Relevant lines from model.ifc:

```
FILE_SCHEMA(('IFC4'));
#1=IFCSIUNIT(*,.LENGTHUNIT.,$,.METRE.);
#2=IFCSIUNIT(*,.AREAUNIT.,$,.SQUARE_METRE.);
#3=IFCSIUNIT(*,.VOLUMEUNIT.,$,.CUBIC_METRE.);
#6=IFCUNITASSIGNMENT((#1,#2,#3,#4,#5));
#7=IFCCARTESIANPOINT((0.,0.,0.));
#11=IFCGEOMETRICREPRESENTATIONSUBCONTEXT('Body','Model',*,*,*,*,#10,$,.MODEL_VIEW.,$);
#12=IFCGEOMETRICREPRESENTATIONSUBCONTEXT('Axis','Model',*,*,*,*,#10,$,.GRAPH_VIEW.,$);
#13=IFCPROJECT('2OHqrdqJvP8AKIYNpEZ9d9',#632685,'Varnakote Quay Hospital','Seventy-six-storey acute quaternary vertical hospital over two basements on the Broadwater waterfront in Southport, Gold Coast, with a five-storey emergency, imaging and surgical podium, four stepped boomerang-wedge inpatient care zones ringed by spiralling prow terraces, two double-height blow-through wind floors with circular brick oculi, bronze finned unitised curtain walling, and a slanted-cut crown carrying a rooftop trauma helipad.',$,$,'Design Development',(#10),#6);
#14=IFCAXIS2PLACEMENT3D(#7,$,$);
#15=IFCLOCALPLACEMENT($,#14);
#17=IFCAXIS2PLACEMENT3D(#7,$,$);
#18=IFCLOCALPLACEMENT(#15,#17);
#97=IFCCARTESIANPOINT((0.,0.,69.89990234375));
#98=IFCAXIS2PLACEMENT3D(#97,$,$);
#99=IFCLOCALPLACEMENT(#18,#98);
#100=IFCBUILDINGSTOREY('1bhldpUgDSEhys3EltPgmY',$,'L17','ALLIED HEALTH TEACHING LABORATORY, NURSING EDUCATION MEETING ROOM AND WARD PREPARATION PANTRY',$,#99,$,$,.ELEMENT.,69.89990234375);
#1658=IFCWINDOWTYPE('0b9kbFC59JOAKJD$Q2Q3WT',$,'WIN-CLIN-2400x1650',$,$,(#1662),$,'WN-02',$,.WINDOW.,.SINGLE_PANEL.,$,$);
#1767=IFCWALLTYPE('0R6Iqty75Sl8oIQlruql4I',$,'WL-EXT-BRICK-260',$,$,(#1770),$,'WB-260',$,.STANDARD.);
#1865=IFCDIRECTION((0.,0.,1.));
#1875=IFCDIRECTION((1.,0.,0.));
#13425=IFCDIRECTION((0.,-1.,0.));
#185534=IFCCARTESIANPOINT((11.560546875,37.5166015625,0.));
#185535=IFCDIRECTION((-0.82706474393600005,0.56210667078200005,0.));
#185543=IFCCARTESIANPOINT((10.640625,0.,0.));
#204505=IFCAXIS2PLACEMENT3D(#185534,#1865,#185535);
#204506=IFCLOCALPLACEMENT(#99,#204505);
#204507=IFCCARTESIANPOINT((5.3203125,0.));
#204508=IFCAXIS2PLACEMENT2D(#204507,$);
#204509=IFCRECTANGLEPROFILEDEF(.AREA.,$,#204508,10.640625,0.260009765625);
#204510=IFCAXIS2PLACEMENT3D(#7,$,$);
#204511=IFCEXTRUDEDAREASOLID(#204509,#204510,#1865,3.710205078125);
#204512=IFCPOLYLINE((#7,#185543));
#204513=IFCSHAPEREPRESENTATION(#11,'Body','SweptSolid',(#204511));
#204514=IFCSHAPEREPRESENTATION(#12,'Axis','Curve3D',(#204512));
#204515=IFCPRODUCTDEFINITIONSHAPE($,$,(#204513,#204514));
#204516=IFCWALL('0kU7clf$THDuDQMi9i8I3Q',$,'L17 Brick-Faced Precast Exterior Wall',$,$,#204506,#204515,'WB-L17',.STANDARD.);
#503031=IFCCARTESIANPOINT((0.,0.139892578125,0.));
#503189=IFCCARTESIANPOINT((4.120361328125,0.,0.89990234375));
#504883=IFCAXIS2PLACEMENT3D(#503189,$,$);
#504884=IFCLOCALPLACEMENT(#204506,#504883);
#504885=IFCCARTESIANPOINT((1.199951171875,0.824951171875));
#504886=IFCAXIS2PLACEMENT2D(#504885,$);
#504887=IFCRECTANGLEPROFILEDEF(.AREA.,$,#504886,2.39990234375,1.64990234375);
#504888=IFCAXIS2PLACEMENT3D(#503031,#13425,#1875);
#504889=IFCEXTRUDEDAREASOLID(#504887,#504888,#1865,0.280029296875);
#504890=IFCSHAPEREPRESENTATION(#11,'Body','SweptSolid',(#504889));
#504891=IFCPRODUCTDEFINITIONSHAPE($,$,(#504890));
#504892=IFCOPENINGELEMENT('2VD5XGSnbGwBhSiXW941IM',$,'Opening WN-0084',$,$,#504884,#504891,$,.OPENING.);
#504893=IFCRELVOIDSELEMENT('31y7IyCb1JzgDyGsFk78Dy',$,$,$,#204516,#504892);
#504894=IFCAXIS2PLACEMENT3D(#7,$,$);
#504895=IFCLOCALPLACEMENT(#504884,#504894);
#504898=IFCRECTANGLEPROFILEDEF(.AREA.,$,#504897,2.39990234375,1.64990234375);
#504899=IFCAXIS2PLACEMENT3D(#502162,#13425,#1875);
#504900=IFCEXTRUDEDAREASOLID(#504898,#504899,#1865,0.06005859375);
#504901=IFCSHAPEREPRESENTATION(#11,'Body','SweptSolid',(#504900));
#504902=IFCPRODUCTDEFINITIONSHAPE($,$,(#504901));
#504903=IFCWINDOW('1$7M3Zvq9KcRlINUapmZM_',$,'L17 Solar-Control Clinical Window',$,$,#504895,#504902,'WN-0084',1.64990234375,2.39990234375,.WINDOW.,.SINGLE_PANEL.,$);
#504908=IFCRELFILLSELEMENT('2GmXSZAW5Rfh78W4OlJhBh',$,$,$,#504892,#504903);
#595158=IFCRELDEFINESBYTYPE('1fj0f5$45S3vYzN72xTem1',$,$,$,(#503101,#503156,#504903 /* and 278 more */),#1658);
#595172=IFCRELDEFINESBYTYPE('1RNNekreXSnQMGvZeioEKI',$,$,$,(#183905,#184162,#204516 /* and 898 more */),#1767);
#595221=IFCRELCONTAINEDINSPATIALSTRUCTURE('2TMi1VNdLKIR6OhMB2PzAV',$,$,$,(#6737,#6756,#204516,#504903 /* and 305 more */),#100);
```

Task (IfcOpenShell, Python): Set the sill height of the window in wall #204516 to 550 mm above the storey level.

```python
import numpy as np
import ifcopenshell
import ifcopenshell.api.geometry
import ifcopenshell.geom
import ifcopenshell.util.element
import ifcopenshell.util.placement
import ifcopenshell.util.shape
import ifcopenshell.util.unit

model = ifcopenshell.open("model.ifc")
unit_scale = ifcopenshell.util.unit.calculate_unit_scale(model)

window = model.by_id(504903)
opening = window.FillsVoids[0].RelatingOpeningElement
storey = ifcopenshell.util.element.get_container(window, ifc_class="IfcBuildingStorey")
level = ifcopenshell.util.placement.get_local_placement(storey.ObjectPlacement)[2, 3]

# The opening's origin need not be at the sill, so measure its lowest point.
shape = ifcopenshell.geom.create_shape(ifcopenshell.geom.settings(), opening)
bottom = ifcopenshell.util.shape.get_shape_bottom_elevation(shape, shape.geometry) / unit_scale
dz = level + 0.55 / unit_scale - bottom

shift = np.array([0.0, 0.0, dz])
# The window is placed relative to its opening, so it follows when the opening moves.
matrix = ifcopenshell.util.placement.get_local_placement(opening.ObjectPlacement)
matrix[:3, 3] += shift
ifcopenshell.api.geometry.edit_object_placement(
    model, product=opening, matrix=matrix, is_si=False, should_transform_children=True
)

print(f"moved by {dz * unit_scale:+.3f} m")

model.write("model-out.ifc")
```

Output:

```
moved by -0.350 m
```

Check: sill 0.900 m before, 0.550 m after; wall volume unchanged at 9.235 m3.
